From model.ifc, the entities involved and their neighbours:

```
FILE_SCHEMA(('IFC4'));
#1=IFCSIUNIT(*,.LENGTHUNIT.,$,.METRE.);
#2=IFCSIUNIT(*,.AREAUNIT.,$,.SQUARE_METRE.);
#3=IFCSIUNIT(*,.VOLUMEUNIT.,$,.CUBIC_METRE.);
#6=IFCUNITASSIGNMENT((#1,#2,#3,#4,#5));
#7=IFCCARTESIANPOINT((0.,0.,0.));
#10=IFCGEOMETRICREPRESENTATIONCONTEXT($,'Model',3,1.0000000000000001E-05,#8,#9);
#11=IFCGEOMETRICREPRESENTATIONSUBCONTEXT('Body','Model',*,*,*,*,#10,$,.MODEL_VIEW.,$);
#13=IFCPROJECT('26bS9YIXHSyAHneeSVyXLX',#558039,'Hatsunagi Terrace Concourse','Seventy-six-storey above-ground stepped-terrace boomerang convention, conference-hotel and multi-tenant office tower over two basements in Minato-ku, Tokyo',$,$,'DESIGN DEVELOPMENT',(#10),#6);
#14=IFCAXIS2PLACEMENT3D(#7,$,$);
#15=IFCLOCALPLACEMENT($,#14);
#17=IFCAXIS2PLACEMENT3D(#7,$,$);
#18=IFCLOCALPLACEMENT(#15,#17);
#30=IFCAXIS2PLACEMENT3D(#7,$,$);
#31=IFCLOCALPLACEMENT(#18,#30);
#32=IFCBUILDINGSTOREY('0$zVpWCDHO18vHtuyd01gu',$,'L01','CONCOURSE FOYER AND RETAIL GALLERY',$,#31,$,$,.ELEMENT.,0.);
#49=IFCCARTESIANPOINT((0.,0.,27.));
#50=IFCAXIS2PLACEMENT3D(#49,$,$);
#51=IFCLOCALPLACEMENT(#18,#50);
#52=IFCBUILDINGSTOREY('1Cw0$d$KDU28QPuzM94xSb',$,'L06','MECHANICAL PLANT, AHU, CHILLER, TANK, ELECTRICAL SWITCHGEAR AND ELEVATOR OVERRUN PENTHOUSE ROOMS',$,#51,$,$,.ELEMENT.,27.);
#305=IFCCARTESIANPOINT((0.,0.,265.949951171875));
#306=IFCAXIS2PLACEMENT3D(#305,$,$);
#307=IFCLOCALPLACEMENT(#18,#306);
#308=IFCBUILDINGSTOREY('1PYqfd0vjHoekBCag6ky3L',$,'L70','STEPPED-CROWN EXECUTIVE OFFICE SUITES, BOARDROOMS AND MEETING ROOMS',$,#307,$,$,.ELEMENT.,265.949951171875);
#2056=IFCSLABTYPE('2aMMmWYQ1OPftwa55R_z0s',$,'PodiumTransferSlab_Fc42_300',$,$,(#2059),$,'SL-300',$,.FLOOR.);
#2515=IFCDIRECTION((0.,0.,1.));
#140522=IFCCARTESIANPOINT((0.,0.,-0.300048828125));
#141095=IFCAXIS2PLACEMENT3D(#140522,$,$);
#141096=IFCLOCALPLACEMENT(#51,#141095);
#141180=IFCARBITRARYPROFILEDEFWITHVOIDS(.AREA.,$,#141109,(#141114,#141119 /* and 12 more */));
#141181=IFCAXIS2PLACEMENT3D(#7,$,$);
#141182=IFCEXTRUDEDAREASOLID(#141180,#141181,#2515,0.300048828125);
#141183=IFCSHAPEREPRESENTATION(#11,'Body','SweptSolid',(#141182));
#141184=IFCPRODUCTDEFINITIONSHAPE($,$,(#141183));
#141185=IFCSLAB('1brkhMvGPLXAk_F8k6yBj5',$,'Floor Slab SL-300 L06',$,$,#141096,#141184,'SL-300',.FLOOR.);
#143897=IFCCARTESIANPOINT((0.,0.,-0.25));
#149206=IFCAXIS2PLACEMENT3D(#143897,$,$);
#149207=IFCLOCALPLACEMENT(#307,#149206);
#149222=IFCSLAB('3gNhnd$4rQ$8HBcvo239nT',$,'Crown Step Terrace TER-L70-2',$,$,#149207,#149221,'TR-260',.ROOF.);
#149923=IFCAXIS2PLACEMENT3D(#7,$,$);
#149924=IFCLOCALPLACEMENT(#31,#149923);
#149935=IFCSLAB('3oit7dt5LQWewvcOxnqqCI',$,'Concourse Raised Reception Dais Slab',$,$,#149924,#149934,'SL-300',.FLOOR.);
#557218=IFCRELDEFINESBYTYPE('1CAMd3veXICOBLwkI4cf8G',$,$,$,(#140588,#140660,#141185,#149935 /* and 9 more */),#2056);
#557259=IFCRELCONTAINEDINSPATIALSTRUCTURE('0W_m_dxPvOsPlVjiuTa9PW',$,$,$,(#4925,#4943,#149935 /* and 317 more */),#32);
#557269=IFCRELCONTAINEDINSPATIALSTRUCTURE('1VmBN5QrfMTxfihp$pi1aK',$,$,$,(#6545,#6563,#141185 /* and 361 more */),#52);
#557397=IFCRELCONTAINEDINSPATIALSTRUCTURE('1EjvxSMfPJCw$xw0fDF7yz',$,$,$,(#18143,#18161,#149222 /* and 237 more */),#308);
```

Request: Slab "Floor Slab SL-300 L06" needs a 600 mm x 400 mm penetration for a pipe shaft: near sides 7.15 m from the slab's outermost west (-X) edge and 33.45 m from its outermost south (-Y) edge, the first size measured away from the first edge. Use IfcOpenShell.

```python
import numpy as np
import ifcopenshell
import ifcopenshell.api.feature
import ifcopenshell.api.geometry
import ifcopenshell.api.root
import ifcopenshell.geom
import ifcopenshell.util.placement
import ifcopenshell.util.representation
import ifcopenshell.util.shape
import ifcopenshell.util.unit

model = ifcopenshell.open("model.ifc")
unit_scale = ifcopenshell.util.unit.calculate_unit_scale(model)
settings = ifcopenshell.geom.settings()


def volume(element):
    """Net volume in cubic metres, openings subtracted."""
    shape = ifcopenshell.geom.create_shape(settings, element)
    return ifcopenshell.util.shape.get_volume(shape.geometry)


slab = model.by_guid("1brkhMvGPLXAk_F8k6yBj5")
before = volume(slab)

# Extent in the slab's own axes, in metres. The edges named are its -X and -Y sides.
slab_shape = ifcopenshell.geom.create_shape(settings, slab)
vertices = ifcopenshell.util.shape.get_vertices(slab_shape.geometry)
x_min, y_min, bottom = vertices.min(axis=0)
top = vertices[:, 2].max()

opening = ifcopenshell.api.root.create_entity(model, ifc_class="IfcOpeningElement", name="Pipe shaft opening", predefined_type="OPENING")
context = ifcopenshell.util.representation.get_context(model, "Model", "Body", "MODEL_VIEW")
width, depth = 0.6, 0.4
outline = [(0.0, 0.0), (width, 0.0), (width, depth), (0.0, depth), (0.0, 0.0)]
# Overshoot both faces by 50 mm so the cut is clean.
shape = ifcopenshell.api.geometry.add_slab_representation(
    model, context=context, depth=top - bottom + 0.1, polyline=outline
)
ifcopenshell.api.geometry.assign_representation(model, product=opening, representation=shape)

matrix = ifcopenshell.util.placement.get_local_placement(slab.ObjectPlacement)
matrix[:, 3] = matrix @ np.append(np.array([x_min + 7.15, y_min + 33.45, bottom - 0.05]) / unit_scale, 1.0)
ifcopenshell.api.geometry.edit_object_placement(model, product=opening, matrix=matrix, is_si=False)
ifcopenshell.api.feature.add_feature(model, feature=opening, element=slab)

after = volume(slab)

print(f"slab volume {before:.3f} -> {after:.3f} m3")

model.write("model_updated.ifc")
```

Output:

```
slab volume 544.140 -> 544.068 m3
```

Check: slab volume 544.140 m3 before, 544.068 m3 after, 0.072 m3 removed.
